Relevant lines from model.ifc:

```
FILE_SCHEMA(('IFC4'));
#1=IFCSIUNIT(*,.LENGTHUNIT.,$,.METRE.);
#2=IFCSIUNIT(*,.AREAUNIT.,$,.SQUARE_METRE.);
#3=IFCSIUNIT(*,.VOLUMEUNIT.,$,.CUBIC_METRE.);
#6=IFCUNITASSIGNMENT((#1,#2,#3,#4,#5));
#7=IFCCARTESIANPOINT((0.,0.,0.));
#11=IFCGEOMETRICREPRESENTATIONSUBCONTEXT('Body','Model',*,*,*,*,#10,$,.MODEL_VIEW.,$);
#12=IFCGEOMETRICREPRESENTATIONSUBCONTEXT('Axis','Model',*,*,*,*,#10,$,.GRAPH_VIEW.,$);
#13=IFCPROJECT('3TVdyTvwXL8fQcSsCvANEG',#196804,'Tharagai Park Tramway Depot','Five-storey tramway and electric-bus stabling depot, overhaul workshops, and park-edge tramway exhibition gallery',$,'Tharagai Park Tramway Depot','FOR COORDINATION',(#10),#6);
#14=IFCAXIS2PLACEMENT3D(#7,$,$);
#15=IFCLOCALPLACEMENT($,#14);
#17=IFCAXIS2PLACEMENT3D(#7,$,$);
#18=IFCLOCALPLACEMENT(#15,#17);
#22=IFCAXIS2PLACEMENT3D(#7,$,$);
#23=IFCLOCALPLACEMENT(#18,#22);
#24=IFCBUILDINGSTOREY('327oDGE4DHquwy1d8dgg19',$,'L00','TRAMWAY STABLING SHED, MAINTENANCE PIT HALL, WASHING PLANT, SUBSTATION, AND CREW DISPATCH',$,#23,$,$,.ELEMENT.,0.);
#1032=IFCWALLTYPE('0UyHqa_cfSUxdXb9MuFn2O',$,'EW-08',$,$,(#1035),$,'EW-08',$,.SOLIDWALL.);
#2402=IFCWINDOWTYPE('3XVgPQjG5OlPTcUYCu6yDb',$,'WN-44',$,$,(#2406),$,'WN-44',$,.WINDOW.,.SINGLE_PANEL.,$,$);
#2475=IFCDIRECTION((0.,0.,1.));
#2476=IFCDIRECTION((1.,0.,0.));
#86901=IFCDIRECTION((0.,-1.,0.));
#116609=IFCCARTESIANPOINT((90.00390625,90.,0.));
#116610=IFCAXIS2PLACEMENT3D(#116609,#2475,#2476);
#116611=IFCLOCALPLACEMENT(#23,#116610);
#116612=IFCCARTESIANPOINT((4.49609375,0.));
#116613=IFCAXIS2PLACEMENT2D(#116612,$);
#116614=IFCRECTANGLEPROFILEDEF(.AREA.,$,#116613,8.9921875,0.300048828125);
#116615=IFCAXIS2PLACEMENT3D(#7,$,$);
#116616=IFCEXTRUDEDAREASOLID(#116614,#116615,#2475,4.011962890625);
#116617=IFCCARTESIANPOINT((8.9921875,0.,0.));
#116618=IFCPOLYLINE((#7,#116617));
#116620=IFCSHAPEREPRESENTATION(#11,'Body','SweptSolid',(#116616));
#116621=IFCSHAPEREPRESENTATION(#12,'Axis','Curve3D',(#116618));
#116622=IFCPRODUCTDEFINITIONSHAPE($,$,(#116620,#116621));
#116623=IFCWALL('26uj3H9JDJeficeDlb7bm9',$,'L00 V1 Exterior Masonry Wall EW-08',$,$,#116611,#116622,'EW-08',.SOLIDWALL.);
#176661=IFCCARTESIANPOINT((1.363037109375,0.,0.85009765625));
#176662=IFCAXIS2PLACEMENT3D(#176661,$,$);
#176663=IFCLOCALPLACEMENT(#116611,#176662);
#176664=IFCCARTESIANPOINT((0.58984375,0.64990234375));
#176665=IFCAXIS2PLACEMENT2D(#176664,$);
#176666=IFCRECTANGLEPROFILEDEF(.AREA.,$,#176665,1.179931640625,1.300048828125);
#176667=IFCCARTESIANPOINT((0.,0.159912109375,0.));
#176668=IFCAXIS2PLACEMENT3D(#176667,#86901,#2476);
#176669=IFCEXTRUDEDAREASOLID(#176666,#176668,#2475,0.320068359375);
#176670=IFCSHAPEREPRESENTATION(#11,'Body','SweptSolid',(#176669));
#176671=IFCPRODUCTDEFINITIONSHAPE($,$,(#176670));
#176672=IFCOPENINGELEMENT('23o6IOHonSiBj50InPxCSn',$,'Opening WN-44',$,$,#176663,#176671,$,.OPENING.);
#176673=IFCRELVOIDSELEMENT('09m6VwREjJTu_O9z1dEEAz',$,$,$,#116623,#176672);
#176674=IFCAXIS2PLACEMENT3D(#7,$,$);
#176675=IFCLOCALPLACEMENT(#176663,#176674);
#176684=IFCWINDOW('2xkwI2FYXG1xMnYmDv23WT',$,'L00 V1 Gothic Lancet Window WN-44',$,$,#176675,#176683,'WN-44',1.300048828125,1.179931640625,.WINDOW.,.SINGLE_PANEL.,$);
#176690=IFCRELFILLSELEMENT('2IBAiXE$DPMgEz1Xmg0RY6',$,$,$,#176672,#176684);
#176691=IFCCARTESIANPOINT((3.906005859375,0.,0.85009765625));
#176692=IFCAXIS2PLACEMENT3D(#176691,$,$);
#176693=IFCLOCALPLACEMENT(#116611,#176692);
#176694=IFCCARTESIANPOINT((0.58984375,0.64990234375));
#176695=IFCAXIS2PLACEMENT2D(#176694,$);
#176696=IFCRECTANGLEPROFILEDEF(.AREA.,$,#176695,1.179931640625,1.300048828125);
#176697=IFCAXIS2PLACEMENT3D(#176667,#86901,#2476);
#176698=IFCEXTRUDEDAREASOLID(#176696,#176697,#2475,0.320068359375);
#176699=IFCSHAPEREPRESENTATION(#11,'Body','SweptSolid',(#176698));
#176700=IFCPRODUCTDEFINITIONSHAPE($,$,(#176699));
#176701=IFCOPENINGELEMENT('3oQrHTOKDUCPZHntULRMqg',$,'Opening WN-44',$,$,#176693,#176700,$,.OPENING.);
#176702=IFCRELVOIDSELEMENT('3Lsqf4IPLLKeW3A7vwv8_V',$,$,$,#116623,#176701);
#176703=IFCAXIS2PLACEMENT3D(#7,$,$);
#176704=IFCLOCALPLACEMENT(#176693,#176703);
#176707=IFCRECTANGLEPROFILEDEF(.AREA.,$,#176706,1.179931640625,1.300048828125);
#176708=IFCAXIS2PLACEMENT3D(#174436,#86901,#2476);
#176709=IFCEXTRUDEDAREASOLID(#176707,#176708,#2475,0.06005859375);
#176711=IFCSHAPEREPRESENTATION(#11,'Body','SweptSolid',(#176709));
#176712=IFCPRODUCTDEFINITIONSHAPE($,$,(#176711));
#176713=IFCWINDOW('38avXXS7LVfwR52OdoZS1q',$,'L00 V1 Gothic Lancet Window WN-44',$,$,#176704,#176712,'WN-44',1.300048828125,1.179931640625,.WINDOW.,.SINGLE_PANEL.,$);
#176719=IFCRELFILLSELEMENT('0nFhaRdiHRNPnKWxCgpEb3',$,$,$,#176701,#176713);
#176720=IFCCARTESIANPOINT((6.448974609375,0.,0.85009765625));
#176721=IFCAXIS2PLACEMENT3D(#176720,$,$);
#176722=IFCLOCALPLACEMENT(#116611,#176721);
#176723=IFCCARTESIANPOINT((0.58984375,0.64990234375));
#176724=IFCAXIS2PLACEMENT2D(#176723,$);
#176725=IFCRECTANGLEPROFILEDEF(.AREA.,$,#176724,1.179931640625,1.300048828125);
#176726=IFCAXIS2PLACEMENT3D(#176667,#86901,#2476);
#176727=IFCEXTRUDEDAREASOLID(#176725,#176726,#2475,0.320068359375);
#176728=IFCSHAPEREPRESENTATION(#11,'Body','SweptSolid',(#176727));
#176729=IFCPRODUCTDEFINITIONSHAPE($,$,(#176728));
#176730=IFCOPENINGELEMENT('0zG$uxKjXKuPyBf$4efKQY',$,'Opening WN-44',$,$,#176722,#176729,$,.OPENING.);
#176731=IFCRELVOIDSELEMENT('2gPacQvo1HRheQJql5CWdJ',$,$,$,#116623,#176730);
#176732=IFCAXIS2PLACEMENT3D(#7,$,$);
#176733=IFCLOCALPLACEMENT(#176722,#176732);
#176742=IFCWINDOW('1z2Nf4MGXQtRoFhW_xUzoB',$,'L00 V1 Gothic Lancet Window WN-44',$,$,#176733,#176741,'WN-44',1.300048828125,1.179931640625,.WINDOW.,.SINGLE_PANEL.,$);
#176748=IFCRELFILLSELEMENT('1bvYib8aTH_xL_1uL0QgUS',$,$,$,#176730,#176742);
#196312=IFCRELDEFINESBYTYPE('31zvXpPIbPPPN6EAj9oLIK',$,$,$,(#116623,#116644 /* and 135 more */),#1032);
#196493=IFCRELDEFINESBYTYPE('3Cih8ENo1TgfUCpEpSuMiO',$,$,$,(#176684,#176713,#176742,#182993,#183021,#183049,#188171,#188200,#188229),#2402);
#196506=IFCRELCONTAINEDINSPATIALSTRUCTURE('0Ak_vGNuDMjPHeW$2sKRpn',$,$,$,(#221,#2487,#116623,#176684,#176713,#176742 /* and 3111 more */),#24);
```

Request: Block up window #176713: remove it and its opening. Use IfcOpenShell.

```python
import ifcopenshell
import ifcopenshell.api.feature
import ifcopenshell.api.root
import ifcopenshell.geom
import ifcopenshell.util.shape

model = ifcopenshell.open("model.ifc")
settings = ifcopenshell.geom.settings()


def volume(element):
    """Net volume in cubic metres, openings subtracted."""
    shape = ifcopenshell.geom.create_shape(settings, element)
    return ifcopenshell.util.shape.get_volume(shape.geometry)


window = model.by_id(176713)
opening = window.FillsVoids[0].RelatingOpeningElement
wall = opening.VoidsElements[0].RelatingBuildingElement
before = volume(wall)

ifcopenshell.api.root.remove_product(model, product=window)
ifcopenshell.api.feature.remove_feature(model, feature=opening)

after = volume(wall)

print(f"wall volume {before:.3f} -> {after:.3f} m3")

model.write("model_rev.ifc")
```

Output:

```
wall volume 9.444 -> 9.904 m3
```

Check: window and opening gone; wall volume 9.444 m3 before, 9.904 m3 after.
